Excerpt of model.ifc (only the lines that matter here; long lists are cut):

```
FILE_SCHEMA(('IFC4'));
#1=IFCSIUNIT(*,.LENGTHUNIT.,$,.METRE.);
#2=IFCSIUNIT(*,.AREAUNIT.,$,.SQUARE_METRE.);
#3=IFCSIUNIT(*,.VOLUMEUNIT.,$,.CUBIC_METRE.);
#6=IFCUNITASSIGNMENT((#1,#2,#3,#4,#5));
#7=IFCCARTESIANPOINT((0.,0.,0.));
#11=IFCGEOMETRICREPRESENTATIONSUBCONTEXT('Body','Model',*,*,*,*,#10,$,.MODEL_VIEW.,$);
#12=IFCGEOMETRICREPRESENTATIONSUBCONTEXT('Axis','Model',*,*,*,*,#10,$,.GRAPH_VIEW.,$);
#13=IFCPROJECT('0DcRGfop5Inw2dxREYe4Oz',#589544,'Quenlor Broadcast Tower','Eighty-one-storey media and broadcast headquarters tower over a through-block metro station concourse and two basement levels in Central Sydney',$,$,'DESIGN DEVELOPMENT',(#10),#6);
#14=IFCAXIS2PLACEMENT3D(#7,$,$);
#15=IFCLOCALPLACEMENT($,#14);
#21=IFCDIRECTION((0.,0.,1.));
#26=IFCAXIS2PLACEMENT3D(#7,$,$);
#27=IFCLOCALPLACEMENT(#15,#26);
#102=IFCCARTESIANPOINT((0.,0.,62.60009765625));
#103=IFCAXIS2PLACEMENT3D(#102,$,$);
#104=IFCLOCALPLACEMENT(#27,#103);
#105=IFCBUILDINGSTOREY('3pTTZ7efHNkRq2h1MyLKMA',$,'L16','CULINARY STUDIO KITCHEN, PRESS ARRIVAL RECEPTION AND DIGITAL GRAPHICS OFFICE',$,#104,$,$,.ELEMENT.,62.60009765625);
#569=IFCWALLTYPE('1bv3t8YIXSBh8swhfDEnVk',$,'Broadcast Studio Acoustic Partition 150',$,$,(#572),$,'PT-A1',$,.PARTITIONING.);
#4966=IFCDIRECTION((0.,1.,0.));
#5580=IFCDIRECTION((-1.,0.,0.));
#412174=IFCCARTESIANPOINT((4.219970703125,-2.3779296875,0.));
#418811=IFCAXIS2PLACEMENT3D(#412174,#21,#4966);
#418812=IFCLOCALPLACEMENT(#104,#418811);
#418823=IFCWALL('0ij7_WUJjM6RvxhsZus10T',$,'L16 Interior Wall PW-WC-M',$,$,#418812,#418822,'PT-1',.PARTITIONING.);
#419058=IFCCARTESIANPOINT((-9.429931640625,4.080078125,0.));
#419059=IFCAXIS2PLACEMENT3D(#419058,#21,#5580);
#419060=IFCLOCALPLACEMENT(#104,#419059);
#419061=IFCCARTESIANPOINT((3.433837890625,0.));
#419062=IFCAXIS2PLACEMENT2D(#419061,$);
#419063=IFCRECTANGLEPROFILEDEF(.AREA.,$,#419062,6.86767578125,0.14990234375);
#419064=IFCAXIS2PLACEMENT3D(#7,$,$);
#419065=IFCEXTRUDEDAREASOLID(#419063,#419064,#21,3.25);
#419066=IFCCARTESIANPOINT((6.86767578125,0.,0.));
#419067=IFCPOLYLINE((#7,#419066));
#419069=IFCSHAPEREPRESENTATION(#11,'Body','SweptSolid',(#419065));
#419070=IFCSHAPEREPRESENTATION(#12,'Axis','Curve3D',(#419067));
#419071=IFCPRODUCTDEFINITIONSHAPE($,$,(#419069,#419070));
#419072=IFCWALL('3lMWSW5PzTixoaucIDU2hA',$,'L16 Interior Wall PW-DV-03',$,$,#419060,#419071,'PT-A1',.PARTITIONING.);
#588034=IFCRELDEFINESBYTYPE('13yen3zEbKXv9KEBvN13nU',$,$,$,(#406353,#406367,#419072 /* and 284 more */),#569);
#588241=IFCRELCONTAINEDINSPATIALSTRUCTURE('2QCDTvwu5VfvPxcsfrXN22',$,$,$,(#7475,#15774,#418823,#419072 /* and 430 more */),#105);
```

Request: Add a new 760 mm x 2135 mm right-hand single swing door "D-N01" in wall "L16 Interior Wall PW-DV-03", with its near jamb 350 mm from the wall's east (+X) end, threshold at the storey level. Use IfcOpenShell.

```python
import numpy as np
import ifcopenshell
import ifcopenshell.api.feature
import ifcopenshell.api.geometry
import ifcopenshell.api.root
import ifcopenshell.api.spatial
import ifcopenshell.geom
import ifcopenshell.util.element
import ifcopenshell.util.placement
import ifcopenshell.util.representation
import ifcopenshell.util.shape
import ifcopenshell.util.unit

model = ifcopenshell.open("model.ifc")
unit_scale = ifcopenshell.util.unit.calculate_unit_scale(model)
settings = ifcopenshell.geom.settings()


def volume(element):
    """Net volume in cubic metres, openings subtracted."""
    shape = ifcopenshell.geom.create_shape(settings, element)
    return ifcopenshell.util.shape.get_volume(shape.geometry)


wall = model.by_id(419072)
storey = ifcopenshell.util.element.get_container(wall, ifc_class="IfcBuildingStorey")
context = ifcopenshell.util.representation.get_context(model, "Model", "Body", "MODEL_VIEW")
before = volume(wall)

width, height, from_end, sill = 0.76, 2.135, 0.35, 0.0  # metres

# The wall runs along its own X axis, and the end named is its -X end.
wall_shape = ifcopenshell.geom.create_shape(settings, wall)
x, y, z = ifcopenshell.util.shape.get_vertices(wall_shape.geometry).T
start = x.min() + from_end
face, thickness = float(y.min()), float(y.max() - y.min())
wall_matrix = ifcopenshell.util.placement.get_local_placement(wall.ObjectPlacement)
level = ifcopenshell.util.placement.get_local_placement(storey.ObjectPlacement)[2, 3]


def in_wall(x, y):
    """Placement at x, y metres in the wall's axes, at sill height."""
    matrix = wall_matrix.copy()
    matrix[:, 3] = wall_matrix @ np.array([x / unit_scale, y / unit_scale, 0.0, 1.0])
    matrix[2, 3] = level + sill / unit_scale
    return matrix


# Opening: a box that overshoots both wall faces by 50 mm.
opening = ifcopenshell.api.root.create_entity(model, ifc_class="IfcOpeningElement", predefined_type="OPENING")
box = ifcopenshell.api.geometry.add_wall_representation(
    model, context=context, length=width, height=height, thickness=thickness + 0.1
)
ifcopenshell.api.geometry.assign_representation(model, product=opening, representation=box)
ifcopenshell.api.geometry.edit_object_placement(model, product=opening, matrix=in_wall(start, face - 0.05), is_si=False)
ifcopenshell.api.feature.add_feature(model, feature=opening, element=wall)

door = ifcopenshell.api.root.create_entity(model, ifc_class="IfcDoor", name="D-N01", predefined_type="DOOR")
door.OverallWidth, door.OverallHeight = width / unit_scale, height / unit_scale
door.OperationType = "SINGLE_SWING_RIGHT"
body = ifcopenshell.api.geometry.add_door_representation(
    model,
    context=context,
    overall_width=door.OverallWidth,
    overall_height=door.OverallHeight,
    operation_type="SINGLE_SWING_RIGHT",
    lining_properties={"LiningDepth": thickness / unit_scale, "ThresholdDepth": thickness / unit_scale},
)
ifcopenshell.api.geometry.assign_representation(model, product=door, representation=body)
ifcopenshell.api.spatial.assign_container(model, products=[door], relating_structure=storey)
ifcopenshell.api.feature.add_filling(model, opening=opening, element=door)

# The lining spans the wall, so the door starts at the wall face.
ifcopenshell.api.geometry.edit_object_placement(model, product=door, matrix=in_wall(start, face), is_si=False)

after = volume(wall)

print(f"wall volume {before:.3f} -> {after:.3f} m3")

model.write("model_edited.ifc")
```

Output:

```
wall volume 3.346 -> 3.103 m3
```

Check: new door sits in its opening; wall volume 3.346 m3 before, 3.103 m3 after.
